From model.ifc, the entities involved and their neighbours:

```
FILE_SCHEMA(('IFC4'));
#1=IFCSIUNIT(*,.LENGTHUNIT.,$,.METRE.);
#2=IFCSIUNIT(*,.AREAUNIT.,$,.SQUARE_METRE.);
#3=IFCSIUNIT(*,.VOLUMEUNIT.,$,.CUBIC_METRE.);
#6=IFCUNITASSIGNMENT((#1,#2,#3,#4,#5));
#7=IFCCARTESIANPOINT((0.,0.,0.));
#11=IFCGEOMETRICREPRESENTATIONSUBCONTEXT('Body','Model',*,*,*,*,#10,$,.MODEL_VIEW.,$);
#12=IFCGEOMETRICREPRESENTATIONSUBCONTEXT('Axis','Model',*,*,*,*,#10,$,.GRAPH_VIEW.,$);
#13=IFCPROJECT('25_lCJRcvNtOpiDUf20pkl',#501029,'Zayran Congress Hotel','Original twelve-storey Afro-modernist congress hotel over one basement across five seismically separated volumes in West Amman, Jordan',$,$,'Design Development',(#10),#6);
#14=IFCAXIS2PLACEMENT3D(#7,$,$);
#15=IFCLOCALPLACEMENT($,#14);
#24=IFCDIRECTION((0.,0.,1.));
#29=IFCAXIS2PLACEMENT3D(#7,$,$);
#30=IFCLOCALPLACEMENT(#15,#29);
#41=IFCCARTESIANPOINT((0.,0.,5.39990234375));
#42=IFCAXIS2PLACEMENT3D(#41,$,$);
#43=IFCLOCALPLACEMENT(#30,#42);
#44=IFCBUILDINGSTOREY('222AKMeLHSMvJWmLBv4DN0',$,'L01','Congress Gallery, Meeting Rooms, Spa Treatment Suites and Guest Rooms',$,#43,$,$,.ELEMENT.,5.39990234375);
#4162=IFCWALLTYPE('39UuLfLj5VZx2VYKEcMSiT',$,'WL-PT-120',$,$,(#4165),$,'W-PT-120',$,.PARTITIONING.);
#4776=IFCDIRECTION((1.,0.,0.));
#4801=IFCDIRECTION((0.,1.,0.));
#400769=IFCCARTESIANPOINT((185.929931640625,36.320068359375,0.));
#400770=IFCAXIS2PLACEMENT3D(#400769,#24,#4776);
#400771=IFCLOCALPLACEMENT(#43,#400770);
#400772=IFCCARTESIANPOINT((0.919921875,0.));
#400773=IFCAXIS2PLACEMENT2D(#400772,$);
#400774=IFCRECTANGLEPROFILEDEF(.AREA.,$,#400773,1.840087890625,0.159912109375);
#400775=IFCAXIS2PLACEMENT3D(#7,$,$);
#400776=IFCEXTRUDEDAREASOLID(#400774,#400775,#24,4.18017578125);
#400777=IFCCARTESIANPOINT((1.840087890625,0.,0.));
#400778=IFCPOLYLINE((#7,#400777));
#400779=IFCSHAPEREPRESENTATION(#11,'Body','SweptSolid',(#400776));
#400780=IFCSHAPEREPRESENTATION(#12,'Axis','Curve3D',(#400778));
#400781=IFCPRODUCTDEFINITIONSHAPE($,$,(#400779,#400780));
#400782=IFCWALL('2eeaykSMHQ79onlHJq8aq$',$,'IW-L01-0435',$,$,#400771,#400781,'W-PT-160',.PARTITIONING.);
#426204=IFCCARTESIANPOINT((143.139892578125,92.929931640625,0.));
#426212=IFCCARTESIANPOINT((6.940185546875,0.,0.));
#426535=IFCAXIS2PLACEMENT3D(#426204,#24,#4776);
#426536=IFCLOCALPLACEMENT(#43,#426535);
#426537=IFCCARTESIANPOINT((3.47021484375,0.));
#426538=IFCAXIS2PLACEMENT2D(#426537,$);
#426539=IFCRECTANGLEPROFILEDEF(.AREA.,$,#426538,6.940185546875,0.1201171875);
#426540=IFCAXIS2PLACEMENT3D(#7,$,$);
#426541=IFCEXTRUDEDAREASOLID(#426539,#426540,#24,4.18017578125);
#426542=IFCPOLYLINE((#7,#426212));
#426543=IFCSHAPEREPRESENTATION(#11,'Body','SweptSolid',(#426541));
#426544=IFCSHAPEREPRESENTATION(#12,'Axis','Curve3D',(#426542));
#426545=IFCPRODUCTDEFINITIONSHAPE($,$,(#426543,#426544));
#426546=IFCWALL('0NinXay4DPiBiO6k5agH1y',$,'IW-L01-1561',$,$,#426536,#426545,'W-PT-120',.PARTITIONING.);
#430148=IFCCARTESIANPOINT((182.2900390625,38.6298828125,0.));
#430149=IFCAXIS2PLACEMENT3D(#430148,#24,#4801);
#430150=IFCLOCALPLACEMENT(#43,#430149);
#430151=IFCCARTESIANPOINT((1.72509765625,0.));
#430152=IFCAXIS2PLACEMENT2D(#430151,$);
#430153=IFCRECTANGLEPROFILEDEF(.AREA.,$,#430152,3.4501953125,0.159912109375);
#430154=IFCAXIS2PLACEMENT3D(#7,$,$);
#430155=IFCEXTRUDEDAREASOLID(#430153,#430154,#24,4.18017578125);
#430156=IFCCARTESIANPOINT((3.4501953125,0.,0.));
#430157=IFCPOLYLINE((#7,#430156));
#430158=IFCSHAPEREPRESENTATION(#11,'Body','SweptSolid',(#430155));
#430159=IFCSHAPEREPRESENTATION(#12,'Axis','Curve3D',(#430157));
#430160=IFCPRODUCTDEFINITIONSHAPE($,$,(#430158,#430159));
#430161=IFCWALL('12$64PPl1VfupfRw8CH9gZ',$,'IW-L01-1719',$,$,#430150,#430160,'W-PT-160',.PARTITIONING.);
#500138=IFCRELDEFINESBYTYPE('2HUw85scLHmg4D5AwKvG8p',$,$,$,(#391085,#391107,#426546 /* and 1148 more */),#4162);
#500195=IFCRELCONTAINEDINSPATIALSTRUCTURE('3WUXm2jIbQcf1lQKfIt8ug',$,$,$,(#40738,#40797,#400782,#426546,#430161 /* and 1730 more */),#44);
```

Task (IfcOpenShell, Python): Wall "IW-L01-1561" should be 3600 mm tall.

```python
import ifcopenshell
import ifcopenshell.geom
import ifcopenshell.util.representation
import ifcopenshell.util.shape

model = ifcopenshell.open("model.ifc")
settings = ifcopenshell.geom.settings()


def volume(element):
    """Net volume in cubic metres, openings subtracted."""
    shape = ifcopenshell.geom.create_shape(settings, element)
    return ifcopenshell.util.shape.get_volume(shape.geometry)


wall = model.by_guid("0NinXay4DPiBiO6k5agH1y")
before = volume(wall)

body = ifcopenshell.util.representation.get_representation(wall, "Model", "Body")
solid = body.Items[0]
old_height = solid.Depth
solid.Depth = 3.6
after = volume(wall)

print(f"height {old_height:g} -> {solid.Depth:g}, volume {before:.3f} -> {after:.3f} m3")

model.write("model_rev.ifc")
```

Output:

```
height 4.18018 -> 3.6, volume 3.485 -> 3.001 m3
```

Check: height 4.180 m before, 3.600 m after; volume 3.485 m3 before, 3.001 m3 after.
